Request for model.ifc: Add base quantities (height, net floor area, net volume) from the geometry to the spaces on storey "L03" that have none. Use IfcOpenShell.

First a look at what the model holds.

```python
import ifcopenshell
import ifcopenshell.util.element
import ifcopenshell.util.unit

model = ifcopenshell.open("model.ifc")
print(model.schema)
for unit_type in ("LENGTHUNIT", "AREAUNIT", "VOLUMEUNIT"):
    print(unit_type, ifcopenshell.util.unit.calculate_unit_scale(model, unit_type))
storey = next(s for s in model.by_type("IfcBuildingStorey") if s.Name == "L03")
spaces = [e for e in ifcopenshell.util.element.get_decomposition(storey) if e.is_a("IfcSpace")]
for e in sorted(spaces, key=lambda e: e.id()):
    print(e.id(), e.is_a(), e.Name, list(ifcopenshell.util.element.get_psets(e, qtos_only=True)), sep=" | ")
```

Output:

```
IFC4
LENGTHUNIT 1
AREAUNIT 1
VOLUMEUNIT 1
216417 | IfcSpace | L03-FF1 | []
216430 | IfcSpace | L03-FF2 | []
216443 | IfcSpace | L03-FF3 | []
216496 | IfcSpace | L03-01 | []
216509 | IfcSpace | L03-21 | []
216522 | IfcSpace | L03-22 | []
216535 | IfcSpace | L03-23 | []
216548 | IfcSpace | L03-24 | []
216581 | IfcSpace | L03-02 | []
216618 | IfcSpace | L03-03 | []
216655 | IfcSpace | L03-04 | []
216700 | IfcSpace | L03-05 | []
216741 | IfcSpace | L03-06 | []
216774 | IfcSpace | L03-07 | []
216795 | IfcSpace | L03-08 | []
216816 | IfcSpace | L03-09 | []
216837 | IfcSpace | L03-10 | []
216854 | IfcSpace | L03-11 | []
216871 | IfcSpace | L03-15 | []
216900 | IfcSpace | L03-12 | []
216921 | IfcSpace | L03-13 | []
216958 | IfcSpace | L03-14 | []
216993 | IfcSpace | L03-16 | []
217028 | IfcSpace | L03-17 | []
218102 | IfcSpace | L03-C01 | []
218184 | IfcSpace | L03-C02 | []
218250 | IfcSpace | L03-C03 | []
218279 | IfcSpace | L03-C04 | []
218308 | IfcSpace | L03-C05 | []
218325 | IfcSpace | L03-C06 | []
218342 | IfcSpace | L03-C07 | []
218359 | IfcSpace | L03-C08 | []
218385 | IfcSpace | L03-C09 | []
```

```python
import ifcopenshell
import ifcopenshell.api.pset
import ifcopenshell.geom
import ifcopenshell.util.element
import ifcopenshell.util.shape
import ifcopenshell.util.unit

model = ifcopenshell.open("model.ifc")
unit_scale = ifcopenshell.util.unit.calculate_unit_scale(model)
area_scale = ifcopenshell.util.unit.calculate_unit_scale(model, "AREAUNIT")
volume_scale = ifcopenshell.util.unit.calculate_unit_scale(model, "VOLUMEUNIT")
settings = ifcopenshell.geom.settings()

storey = next(s for s in model.by_type("IfcBuildingStorey") if s.Name == "L03")
spaces = [e for e in ifcopenshell.util.element.get_decomposition(storey) if e.is_a("IfcSpace")]

for e in sorted(spaces, key=lambda e: e.id()):
    if ifcopenshell.util.element.get_psets(e, qtos_only=True, should_inherit=False):
        continue
    # Geometry comes back in metres, in the element's own axes.
    shape = ifcopenshell.geom.create_shape(settings, e)
    values = {
        "Height": ifcopenshell.util.shape.get_z(shape.geometry) / unit_scale,
        "NetFloorArea": ifcopenshell.util.shape.get_footprint_area(shape.geometry) / area_scale,
        "NetVolume": ifcopenshell.util.shape.get_volume(shape.geometry) / volume_scale,
    }
    qto = ifcopenshell.api.pset.add_qto(model, product=e, name="Qto_SpaceBaseQuantities")
    ifcopenshell.api.pset.edit_qto(model, qto=qto, properties=values)
    print(e.id(), {k: round(v, 3) for k, v in values.items()})

model.write("model_v2.ifc")
```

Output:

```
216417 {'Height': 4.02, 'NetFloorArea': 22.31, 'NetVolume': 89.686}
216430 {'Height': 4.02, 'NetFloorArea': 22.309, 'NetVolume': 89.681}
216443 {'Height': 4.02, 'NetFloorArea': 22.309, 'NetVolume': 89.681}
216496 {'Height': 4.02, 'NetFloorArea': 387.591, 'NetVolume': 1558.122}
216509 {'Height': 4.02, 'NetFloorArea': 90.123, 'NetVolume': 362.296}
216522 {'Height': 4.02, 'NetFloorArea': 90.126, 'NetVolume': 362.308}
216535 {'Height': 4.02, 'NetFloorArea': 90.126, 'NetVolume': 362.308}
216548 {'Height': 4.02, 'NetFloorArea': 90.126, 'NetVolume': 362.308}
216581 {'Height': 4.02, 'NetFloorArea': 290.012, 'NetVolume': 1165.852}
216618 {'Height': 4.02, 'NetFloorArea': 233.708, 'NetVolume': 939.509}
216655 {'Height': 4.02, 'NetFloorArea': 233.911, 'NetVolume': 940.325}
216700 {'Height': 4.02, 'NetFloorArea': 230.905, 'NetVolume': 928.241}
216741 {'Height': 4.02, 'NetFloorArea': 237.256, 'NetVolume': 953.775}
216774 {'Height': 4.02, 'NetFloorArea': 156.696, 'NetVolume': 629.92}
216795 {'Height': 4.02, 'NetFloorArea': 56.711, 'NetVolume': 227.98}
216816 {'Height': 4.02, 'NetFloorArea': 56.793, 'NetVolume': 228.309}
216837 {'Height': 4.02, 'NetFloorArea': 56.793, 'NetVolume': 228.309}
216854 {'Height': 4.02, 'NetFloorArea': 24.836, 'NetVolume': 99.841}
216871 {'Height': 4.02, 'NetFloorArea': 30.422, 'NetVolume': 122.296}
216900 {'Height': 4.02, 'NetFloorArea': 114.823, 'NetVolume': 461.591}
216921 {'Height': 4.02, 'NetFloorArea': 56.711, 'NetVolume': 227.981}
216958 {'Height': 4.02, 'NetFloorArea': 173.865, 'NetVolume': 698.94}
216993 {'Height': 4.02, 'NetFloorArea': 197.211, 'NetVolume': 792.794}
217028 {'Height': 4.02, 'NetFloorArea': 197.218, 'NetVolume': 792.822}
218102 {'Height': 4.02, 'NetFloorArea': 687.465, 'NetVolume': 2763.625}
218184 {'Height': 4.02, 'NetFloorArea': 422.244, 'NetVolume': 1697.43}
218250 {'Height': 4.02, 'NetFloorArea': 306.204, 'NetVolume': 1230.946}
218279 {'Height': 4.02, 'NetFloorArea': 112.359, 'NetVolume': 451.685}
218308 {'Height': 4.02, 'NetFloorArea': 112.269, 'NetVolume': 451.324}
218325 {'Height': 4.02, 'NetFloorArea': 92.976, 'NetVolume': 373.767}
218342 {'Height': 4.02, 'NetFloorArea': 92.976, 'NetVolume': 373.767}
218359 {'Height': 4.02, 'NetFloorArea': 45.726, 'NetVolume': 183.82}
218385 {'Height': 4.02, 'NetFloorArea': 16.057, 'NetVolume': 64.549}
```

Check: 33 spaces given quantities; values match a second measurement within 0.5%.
